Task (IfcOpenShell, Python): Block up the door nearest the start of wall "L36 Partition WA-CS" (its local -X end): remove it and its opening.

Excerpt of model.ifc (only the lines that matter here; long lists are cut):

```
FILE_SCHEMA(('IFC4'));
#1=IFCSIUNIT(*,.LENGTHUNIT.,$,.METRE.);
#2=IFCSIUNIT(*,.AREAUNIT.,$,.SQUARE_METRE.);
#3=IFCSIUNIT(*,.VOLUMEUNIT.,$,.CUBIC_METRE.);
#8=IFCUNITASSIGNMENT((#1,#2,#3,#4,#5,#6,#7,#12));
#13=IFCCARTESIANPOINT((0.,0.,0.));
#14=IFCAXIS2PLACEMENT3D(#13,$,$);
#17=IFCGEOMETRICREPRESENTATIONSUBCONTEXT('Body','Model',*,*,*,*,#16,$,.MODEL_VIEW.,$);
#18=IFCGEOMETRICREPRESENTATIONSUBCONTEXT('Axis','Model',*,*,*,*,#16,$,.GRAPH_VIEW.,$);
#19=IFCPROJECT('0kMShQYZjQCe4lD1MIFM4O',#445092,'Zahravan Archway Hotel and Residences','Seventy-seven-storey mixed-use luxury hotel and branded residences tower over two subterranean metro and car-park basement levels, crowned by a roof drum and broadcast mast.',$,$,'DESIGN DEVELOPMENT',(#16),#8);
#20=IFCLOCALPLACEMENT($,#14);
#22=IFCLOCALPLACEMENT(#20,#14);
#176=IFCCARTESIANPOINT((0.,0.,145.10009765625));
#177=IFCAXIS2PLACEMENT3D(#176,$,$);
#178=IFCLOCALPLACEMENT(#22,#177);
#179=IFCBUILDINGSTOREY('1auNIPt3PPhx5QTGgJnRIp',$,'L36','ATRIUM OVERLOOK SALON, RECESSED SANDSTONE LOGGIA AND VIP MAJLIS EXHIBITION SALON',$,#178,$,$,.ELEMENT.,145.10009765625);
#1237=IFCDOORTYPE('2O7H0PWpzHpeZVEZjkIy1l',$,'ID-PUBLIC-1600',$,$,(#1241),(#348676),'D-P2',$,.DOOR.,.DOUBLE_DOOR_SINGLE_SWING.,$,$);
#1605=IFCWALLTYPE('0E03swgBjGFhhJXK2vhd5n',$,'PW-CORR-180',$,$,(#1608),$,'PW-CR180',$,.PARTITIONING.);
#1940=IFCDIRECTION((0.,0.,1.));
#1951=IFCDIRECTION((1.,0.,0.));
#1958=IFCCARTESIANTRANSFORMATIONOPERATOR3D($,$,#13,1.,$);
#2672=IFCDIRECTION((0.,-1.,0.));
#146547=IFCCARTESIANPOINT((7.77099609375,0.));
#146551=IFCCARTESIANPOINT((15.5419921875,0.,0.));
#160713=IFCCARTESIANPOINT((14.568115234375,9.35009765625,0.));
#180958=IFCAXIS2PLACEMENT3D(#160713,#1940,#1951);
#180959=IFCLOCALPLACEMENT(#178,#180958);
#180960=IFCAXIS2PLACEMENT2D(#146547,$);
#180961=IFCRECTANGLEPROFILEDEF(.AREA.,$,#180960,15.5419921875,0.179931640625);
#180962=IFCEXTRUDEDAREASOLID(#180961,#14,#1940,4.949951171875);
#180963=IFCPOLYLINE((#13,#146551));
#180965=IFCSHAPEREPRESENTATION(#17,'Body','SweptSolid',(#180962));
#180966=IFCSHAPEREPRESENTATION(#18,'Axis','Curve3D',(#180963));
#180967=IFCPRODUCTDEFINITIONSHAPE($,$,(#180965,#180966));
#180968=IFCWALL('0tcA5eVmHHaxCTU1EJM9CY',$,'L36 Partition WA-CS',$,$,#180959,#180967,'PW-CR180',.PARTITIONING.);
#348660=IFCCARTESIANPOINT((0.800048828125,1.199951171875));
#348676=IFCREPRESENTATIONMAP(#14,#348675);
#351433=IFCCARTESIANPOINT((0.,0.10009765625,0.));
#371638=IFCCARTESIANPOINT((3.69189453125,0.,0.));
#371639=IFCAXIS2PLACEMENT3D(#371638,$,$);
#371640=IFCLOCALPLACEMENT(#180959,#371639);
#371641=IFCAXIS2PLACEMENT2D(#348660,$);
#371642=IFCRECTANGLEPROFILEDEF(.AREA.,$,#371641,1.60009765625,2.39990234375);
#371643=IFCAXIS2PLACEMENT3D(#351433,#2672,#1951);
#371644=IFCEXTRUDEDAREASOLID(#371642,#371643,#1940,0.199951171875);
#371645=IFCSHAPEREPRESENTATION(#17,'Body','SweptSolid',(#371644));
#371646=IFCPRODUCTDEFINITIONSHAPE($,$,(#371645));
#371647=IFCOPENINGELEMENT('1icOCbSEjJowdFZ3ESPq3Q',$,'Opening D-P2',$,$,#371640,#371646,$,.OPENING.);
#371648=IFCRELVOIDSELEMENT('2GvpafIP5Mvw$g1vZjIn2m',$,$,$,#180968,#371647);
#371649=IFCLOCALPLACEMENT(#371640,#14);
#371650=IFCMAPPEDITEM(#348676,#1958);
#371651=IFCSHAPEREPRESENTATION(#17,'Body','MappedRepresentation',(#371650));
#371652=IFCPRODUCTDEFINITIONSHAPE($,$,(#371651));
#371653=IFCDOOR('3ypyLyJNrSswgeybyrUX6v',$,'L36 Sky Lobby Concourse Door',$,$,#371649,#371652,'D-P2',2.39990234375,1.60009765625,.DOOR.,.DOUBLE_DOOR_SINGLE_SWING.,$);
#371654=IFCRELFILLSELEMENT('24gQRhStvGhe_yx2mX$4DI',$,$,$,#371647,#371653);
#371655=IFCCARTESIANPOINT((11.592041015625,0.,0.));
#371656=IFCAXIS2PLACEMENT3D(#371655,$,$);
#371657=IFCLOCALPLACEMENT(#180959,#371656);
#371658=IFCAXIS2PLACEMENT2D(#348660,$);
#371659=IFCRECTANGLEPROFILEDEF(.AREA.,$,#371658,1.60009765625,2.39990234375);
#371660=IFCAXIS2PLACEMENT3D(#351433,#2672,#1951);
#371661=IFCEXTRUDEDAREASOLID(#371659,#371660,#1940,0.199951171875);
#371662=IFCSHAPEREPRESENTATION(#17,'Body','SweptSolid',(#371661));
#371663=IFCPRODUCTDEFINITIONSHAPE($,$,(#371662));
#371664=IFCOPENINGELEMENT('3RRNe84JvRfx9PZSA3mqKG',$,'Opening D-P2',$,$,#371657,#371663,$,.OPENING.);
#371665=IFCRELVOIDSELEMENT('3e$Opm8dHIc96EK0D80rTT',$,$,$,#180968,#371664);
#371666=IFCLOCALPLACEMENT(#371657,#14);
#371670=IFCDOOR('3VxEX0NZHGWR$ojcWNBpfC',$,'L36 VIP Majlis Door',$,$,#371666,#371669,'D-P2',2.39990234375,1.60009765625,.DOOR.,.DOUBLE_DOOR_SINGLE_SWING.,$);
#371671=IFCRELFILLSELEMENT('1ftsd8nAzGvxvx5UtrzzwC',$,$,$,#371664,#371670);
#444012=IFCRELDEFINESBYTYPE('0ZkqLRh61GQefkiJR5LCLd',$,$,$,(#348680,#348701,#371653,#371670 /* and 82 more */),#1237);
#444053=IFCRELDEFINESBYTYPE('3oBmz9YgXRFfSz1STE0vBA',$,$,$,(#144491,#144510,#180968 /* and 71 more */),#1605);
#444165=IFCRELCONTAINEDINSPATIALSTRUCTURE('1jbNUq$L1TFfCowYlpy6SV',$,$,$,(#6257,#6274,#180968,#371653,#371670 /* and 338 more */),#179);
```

```python
import ifcopenshell
import ifcopenshell.api.feature
import ifcopenshell.api.root
import ifcopenshell.geom
import ifcopenshell.util.shape

model = ifcopenshell.open("model.ifc")
settings = ifcopenshell.geom.settings()


def volume(element):
    """Net volume in cubic metres, openings subtracted."""
    shape = ifcopenshell.geom.create_shape(settings, element)
    return ifcopenshell.util.shape.get_volume(shape.geometry)


door = model.by_guid("3ypyLyJNrSswgeybyrUX6v")
opening = door.FillsVoids[0].RelatingOpeningElement
wall = opening.VoidsElements[0].RelatingBuildingElement
before = volume(wall)

ifcopenshell.api.root.remove_product(model, product=door)
ifcopenshell.api.feature.remove_feature(model, feature=opening)

after = volume(wall)

print(f"wall volume {before:.3f} -> {after:.3f} m3")

model.write("model-out.ifc")
```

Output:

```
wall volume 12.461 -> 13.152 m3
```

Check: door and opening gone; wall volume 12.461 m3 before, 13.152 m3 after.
